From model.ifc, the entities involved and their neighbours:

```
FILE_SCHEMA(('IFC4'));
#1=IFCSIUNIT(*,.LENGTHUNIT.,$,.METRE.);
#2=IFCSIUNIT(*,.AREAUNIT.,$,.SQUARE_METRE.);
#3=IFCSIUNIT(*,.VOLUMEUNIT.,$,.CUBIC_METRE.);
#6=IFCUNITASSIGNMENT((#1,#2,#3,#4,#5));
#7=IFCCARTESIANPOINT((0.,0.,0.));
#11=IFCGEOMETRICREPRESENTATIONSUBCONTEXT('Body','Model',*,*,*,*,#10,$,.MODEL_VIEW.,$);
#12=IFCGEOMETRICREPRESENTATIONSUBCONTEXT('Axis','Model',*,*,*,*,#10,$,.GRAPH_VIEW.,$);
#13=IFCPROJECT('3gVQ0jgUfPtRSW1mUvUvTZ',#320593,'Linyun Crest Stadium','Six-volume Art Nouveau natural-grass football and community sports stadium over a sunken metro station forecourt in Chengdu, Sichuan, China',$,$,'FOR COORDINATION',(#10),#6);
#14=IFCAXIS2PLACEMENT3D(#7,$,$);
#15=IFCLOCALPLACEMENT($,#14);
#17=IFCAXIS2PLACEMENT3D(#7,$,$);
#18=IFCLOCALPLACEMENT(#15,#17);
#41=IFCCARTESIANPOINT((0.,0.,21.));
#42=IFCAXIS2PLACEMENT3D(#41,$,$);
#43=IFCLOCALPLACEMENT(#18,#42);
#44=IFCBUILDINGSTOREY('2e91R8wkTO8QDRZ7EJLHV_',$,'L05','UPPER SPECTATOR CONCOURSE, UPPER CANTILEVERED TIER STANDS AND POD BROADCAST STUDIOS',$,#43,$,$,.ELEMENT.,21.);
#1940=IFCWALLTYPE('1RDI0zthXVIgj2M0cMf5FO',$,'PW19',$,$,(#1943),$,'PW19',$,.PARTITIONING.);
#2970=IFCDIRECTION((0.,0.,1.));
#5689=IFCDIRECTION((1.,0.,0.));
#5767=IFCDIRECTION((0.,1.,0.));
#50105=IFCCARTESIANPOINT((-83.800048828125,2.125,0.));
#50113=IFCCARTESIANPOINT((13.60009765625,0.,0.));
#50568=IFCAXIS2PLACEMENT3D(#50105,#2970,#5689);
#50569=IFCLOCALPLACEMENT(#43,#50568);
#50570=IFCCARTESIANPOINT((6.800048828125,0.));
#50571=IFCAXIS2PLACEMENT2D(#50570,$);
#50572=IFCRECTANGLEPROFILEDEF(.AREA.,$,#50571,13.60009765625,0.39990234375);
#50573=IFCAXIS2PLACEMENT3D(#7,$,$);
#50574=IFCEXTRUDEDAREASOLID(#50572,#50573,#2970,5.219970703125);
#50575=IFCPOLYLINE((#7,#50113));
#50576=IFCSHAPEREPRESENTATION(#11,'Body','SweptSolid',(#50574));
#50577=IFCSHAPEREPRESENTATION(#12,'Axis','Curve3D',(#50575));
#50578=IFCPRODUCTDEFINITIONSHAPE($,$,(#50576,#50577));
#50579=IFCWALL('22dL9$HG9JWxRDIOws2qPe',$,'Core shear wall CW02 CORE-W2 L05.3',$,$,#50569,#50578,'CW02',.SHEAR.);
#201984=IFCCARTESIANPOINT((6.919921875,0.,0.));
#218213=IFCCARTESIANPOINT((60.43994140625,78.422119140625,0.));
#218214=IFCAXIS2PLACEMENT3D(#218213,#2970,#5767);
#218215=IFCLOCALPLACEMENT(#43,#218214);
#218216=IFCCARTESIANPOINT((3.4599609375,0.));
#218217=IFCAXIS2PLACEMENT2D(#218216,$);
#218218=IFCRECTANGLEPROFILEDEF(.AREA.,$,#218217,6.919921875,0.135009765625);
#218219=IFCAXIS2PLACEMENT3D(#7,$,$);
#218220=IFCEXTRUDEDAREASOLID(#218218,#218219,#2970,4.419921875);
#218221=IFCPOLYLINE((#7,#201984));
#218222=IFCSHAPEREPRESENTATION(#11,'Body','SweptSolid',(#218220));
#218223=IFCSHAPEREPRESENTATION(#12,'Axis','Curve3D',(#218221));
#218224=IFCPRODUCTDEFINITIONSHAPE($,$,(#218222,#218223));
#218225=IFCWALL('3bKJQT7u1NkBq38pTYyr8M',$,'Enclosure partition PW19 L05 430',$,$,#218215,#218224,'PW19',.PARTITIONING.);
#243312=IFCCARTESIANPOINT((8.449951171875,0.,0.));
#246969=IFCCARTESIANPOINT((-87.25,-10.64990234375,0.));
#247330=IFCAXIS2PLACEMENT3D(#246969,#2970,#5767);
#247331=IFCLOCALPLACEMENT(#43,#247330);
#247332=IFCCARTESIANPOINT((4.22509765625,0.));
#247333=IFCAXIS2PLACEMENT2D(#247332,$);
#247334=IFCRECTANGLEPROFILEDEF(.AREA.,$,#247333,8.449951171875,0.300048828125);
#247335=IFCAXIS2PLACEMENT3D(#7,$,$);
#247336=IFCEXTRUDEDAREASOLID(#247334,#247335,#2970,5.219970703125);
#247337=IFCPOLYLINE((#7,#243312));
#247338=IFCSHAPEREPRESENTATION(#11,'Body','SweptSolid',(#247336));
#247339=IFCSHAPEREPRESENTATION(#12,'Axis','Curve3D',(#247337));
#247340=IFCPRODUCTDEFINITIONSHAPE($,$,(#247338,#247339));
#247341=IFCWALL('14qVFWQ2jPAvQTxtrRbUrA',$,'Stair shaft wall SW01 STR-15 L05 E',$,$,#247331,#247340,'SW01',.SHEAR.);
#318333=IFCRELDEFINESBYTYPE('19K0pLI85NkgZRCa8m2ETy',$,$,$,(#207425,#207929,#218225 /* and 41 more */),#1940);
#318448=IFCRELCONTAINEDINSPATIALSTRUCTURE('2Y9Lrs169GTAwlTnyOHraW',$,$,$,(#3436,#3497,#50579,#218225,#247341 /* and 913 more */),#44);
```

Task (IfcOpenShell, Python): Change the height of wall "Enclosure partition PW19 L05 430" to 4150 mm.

```python
import ifcopenshell
import ifcopenshell.geom
import ifcopenshell.util.representation
import ifcopenshell.util.shape

model = ifcopenshell.open("model.ifc")
settings = ifcopenshell.geom.settings()


def volume(element):
    """Net volume in cubic metres, openings subtracted."""
    shape = ifcopenshell.geom.create_shape(settings, element)
    return ifcopenshell.util.shape.get_volume(shape.geometry)


wall = model.by_guid("3bKJQT7u1NkBq38pTYyr8M")
before = volume(wall)

body = ifcopenshell.util.representation.get_representation(wall, "Model", "Body")
solid = body.Items[0]
old_height = solid.Depth
solid.Depth = 4.15
after = volume(wall)

print(f"height {old_height:g} -> {solid.Depth:g}, volume {before:.3f} -> {after:.3f} m3")

model.write("model-out.ifc")
```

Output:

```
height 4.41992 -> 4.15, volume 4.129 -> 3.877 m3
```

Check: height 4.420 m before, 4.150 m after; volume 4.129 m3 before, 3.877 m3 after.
